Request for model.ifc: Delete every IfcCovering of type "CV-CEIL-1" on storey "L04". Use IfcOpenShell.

First a look at what the model holds.

```python
import ifcopenshell
import ifcopenshell.util.element

model = ifcopenshell.open("model.ifc")
print(model.schema)
storey = next(s for s in model.by_type("IfcBuildingStorey") if s.Name == "L04")
coverings = [e for e in ifcopenshell.util.element.get_decomposition(storey) if e.is_a("IfcCovering")]
seen = {}
for e in coverings:
    element_type = ifcopenshell.util.element.get_type(e)
    name = element_type.Name if element_type not in (None, e) else None
    seen[name] = seen.get(name, 0) + 1
for name, count in sorted(seen.items(), key=str):
    print(count, "x", name)
```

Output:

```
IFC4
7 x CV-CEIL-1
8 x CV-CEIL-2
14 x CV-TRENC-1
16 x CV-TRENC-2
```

```python
import ifcopenshell
import ifcopenshell.api.root
import ifcopenshell.util.element

model = ifcopenshell.open("model.ifc")

storey = next(s for s in model.by_type("IfcBuildingStorey") if s.Name == "L04")
coverings = [e for e in ifcopenshell.util.element.get_decomposition(storey) if e.is_a("IfcCovering")]
targets = [e for e in coverings if (t := ifcopenshell.util.element.get_type(e)) not in (None, e) and t.Name == "CV-CEIL-1"]

for e in targets:
    ifcopenshell.api.root.remove_product(model, product=e)
print(len(targets), "removed")

model.write("model_rev.ifc")
```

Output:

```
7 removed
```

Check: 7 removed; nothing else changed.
